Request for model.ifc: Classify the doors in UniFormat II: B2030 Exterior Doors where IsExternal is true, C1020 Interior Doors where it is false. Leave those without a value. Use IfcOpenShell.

First a look at what the model holds.

```python
import ifcopenshell
import ifcopenshell.util.element

model = ifcopenshell.open("model.ifc")
print(model.schema)
print("classifications:", [c.Name for c in model.by_type("IfcClassification")])
values = [ifcopenshell.util.element.get_pset(e, "Pset_DoorCommon", "IsExternal") for e in model.by_type("IfcDoor")]
for value in (True, False, None):
    print("IsExternal", value, values.count(value))
```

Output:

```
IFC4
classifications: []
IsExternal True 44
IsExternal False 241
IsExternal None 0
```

```python
import ifcopenshell
import ifcopenshell.api.classification
import ifcopenshell.util.element

model = ifcopenshell.open("model.ifc")

system = ifcopenshell.api.classification.add_classification(model, classification="UniFormat II")

doors = model.by_type("IfcDoor")
external = {e: ifcopenshell.util.element.get_pset(e, "Pset_DoorCommon", "IsExternal") for e in doors}
for flag, code, name in ((True, "B2030", "Exterior Doors"), (False, "C1020", "Interior Doors")):
    products = [e for e in doors if external[e] is flag]
    ifcopenshell.api.classification.add_reference(
        model, products=products, classification=system, identification=code, name=name
    )
    print(code, len(products))

model.write("model_edited.ifc")
```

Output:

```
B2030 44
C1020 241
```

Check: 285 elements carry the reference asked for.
